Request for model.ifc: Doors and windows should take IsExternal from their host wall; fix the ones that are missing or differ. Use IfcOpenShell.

First a look at what the model holds.

```python
import ifcopenshell
import ifcopenshell.util.element

model = ifcopenshell.open("model.ifc")
print(model.schema)
seen = {}
for e in model.by_type("IfcDoor") + model.by_type("IfcWindow"):
    if not e.FillsVoids:
        continue
    host = e.FillsVoids[0].RelatingOpeningElement.VoidsElements[0].RelatingBuildingElement
    own = ifcopenshell.util.element.get_pset(e, f"Pset_{e.is_a()[3:].removesuffix('StandardCase')}Common", "IsExternal")
    wall = ifcopenshell.util.element.get_pset(host, "Pset_WallCommon", "IsExternal")
    seen[e.is_a(), own, wall] = seen.get((e.is_a(), own, wall), 0) + 1
for (cls, own, wall), count in sorted(seen.items(), key=str):
    print(count, cls, "IsExternal:", own, "| host wall:", wall)
```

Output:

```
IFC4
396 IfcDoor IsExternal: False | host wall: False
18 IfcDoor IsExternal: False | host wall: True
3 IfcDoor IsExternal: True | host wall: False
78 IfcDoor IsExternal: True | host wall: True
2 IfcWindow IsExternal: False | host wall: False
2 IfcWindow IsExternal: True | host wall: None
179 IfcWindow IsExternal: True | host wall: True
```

```python
import ifcopenshell
import ifcopenshell.api.pset
import ifcopenshell.util.element

model = ifcopenshell.open("model.ifc")

count = 0
for ifc_class, pset_name in (("IfcDoor", "Pset_DoorCommon"), ("IfcWindow", "Pset_WindowCommon")):
    for e in model.by_type(ifc_class):
        if not e.FillsVoids:
            continue
        host = e.FillsVoids[0].RelatingOpeningElement.VoidsElements[0].RelatingBuildingElement
        external = ifcopenshell.util.element.get_pset(host, "Pset_WallCommon", "IsExternal")
        if external is None or ifcopenshell.util.element.get_pset(e, pset_name, "IsExternal") == external:
            continue
        pset = ifcopenshell.api.pset.add_pset(model, product=e, name=pset_name)
        ifcopenshell.api.pset.edit_pset(model, pset=pset, properties={"IsExternal": external})
        count += 1

print(count, "updated")

model.write("model_v2.ifc")
```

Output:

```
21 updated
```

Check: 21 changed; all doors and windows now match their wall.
